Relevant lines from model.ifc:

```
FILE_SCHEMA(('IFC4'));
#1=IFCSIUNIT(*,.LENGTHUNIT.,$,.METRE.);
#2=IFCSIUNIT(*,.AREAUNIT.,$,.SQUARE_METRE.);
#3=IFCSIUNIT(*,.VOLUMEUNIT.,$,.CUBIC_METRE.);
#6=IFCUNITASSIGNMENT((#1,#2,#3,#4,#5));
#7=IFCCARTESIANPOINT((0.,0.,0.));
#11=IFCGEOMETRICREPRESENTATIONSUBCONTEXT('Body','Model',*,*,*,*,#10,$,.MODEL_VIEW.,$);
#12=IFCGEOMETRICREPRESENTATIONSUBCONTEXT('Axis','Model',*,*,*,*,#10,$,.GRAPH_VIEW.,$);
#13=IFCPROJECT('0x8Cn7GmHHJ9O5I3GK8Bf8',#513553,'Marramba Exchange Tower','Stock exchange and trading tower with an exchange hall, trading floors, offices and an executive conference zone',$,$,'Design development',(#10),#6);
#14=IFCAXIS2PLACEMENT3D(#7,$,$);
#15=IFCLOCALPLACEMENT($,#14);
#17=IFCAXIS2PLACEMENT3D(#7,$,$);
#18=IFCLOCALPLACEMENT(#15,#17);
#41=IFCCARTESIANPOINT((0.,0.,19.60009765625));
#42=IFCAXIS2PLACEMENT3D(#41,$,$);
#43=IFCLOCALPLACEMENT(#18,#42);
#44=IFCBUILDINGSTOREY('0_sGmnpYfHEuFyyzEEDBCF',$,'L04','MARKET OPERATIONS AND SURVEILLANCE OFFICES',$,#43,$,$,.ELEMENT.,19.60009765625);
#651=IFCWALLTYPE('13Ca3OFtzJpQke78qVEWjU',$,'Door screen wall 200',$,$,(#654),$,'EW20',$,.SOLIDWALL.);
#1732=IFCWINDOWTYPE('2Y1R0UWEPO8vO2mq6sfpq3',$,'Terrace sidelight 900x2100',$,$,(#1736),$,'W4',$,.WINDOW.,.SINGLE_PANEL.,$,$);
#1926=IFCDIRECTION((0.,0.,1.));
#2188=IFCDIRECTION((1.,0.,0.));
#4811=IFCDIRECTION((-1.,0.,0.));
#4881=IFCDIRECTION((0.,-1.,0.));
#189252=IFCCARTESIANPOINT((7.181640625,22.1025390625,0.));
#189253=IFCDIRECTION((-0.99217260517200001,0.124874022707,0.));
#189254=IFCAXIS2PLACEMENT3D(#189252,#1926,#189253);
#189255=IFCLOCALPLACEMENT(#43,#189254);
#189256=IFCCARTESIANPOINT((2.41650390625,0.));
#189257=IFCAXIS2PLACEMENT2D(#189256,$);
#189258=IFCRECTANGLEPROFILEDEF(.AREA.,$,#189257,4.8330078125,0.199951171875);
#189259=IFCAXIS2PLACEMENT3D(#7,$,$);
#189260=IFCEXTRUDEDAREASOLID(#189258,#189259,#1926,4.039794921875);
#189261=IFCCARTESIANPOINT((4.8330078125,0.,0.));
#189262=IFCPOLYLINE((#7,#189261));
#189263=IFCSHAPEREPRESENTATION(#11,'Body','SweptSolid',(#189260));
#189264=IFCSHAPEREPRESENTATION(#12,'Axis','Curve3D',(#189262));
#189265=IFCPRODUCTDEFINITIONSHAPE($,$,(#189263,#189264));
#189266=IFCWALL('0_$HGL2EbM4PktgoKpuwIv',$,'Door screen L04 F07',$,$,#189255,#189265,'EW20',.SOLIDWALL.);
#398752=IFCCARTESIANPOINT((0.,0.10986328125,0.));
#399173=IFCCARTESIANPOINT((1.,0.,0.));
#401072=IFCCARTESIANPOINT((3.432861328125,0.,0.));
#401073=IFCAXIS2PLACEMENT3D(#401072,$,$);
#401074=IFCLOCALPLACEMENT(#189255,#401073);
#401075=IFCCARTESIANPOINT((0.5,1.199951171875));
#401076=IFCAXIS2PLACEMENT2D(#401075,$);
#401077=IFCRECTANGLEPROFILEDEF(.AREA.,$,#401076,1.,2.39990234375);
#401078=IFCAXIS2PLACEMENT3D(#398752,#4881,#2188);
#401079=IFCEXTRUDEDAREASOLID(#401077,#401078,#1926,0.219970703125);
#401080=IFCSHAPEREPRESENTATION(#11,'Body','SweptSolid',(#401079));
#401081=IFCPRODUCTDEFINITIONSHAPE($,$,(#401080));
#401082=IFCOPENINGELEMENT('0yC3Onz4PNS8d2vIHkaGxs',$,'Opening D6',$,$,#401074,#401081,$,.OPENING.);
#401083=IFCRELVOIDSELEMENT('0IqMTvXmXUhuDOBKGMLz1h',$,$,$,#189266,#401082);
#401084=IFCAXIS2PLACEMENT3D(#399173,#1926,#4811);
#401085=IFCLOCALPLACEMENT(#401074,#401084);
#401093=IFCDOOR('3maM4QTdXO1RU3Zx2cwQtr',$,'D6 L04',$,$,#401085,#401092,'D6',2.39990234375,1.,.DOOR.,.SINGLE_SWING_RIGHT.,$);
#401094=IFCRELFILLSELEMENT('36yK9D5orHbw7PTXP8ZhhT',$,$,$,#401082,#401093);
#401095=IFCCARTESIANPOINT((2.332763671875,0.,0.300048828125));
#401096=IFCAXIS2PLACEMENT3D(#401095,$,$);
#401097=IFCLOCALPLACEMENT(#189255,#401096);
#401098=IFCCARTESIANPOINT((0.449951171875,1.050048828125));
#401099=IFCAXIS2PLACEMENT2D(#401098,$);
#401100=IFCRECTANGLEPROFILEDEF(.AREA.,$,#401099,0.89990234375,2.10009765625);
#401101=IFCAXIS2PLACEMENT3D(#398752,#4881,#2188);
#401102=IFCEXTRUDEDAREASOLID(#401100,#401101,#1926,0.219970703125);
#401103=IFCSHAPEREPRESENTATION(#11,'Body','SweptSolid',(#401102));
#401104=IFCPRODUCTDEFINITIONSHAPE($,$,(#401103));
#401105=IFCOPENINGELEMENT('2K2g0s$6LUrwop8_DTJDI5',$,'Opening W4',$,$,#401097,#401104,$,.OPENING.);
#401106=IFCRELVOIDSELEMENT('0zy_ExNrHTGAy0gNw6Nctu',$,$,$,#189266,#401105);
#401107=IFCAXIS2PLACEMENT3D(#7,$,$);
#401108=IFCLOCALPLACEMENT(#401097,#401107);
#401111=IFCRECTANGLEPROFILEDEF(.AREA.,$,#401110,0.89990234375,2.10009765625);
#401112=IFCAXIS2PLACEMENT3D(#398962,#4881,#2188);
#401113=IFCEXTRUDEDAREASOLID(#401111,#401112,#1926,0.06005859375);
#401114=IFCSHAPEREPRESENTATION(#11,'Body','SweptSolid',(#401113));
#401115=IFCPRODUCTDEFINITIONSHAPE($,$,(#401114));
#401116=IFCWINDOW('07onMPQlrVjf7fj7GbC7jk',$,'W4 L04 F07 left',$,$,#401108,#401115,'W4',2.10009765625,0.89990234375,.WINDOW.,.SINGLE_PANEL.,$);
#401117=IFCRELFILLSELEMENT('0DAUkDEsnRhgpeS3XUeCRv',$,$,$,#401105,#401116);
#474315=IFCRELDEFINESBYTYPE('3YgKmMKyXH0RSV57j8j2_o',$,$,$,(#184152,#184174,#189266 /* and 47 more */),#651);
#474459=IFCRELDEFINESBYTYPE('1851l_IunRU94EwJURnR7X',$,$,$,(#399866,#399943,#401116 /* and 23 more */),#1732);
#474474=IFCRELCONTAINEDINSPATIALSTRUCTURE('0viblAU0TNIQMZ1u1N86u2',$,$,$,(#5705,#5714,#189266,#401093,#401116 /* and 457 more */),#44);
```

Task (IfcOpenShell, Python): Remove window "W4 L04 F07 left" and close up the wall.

```python
import ifcopenshell
import ifcopenshell.api.feature
import ifcopenshell.api.root
import ifcopenshell.geom
import ifcopenshell.util.shape

model = ifcopenshell.open("model.ifc")
settings = ifcopenshell.geom.settings()


def volume(element):
    """Net volume in cubic metres, openings subtracted."""
    shape = ifcopenshell.geom.create_shape(settings, element)
    return ifcopenshell.util.shape.get_volume(shape.geometry)


window = model.by_id(401116)
opening = window.FillsVoids[0].RelatingOpeningElement
wall = opening.VoidsElements[0].RelatingBuildingElement
before = volume(wall)

ifcopenshell.api.root.remove_product(model, product=window)
ifcopenshell.api.feature.remove_feature(model, feature=opening)

after = volume(wall)

print(f"wall volume {before:.3f} -> {after:.3f} m3")

model.write("model_rev.ifc")
```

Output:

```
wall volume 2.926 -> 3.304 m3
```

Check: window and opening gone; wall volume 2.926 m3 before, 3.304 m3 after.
